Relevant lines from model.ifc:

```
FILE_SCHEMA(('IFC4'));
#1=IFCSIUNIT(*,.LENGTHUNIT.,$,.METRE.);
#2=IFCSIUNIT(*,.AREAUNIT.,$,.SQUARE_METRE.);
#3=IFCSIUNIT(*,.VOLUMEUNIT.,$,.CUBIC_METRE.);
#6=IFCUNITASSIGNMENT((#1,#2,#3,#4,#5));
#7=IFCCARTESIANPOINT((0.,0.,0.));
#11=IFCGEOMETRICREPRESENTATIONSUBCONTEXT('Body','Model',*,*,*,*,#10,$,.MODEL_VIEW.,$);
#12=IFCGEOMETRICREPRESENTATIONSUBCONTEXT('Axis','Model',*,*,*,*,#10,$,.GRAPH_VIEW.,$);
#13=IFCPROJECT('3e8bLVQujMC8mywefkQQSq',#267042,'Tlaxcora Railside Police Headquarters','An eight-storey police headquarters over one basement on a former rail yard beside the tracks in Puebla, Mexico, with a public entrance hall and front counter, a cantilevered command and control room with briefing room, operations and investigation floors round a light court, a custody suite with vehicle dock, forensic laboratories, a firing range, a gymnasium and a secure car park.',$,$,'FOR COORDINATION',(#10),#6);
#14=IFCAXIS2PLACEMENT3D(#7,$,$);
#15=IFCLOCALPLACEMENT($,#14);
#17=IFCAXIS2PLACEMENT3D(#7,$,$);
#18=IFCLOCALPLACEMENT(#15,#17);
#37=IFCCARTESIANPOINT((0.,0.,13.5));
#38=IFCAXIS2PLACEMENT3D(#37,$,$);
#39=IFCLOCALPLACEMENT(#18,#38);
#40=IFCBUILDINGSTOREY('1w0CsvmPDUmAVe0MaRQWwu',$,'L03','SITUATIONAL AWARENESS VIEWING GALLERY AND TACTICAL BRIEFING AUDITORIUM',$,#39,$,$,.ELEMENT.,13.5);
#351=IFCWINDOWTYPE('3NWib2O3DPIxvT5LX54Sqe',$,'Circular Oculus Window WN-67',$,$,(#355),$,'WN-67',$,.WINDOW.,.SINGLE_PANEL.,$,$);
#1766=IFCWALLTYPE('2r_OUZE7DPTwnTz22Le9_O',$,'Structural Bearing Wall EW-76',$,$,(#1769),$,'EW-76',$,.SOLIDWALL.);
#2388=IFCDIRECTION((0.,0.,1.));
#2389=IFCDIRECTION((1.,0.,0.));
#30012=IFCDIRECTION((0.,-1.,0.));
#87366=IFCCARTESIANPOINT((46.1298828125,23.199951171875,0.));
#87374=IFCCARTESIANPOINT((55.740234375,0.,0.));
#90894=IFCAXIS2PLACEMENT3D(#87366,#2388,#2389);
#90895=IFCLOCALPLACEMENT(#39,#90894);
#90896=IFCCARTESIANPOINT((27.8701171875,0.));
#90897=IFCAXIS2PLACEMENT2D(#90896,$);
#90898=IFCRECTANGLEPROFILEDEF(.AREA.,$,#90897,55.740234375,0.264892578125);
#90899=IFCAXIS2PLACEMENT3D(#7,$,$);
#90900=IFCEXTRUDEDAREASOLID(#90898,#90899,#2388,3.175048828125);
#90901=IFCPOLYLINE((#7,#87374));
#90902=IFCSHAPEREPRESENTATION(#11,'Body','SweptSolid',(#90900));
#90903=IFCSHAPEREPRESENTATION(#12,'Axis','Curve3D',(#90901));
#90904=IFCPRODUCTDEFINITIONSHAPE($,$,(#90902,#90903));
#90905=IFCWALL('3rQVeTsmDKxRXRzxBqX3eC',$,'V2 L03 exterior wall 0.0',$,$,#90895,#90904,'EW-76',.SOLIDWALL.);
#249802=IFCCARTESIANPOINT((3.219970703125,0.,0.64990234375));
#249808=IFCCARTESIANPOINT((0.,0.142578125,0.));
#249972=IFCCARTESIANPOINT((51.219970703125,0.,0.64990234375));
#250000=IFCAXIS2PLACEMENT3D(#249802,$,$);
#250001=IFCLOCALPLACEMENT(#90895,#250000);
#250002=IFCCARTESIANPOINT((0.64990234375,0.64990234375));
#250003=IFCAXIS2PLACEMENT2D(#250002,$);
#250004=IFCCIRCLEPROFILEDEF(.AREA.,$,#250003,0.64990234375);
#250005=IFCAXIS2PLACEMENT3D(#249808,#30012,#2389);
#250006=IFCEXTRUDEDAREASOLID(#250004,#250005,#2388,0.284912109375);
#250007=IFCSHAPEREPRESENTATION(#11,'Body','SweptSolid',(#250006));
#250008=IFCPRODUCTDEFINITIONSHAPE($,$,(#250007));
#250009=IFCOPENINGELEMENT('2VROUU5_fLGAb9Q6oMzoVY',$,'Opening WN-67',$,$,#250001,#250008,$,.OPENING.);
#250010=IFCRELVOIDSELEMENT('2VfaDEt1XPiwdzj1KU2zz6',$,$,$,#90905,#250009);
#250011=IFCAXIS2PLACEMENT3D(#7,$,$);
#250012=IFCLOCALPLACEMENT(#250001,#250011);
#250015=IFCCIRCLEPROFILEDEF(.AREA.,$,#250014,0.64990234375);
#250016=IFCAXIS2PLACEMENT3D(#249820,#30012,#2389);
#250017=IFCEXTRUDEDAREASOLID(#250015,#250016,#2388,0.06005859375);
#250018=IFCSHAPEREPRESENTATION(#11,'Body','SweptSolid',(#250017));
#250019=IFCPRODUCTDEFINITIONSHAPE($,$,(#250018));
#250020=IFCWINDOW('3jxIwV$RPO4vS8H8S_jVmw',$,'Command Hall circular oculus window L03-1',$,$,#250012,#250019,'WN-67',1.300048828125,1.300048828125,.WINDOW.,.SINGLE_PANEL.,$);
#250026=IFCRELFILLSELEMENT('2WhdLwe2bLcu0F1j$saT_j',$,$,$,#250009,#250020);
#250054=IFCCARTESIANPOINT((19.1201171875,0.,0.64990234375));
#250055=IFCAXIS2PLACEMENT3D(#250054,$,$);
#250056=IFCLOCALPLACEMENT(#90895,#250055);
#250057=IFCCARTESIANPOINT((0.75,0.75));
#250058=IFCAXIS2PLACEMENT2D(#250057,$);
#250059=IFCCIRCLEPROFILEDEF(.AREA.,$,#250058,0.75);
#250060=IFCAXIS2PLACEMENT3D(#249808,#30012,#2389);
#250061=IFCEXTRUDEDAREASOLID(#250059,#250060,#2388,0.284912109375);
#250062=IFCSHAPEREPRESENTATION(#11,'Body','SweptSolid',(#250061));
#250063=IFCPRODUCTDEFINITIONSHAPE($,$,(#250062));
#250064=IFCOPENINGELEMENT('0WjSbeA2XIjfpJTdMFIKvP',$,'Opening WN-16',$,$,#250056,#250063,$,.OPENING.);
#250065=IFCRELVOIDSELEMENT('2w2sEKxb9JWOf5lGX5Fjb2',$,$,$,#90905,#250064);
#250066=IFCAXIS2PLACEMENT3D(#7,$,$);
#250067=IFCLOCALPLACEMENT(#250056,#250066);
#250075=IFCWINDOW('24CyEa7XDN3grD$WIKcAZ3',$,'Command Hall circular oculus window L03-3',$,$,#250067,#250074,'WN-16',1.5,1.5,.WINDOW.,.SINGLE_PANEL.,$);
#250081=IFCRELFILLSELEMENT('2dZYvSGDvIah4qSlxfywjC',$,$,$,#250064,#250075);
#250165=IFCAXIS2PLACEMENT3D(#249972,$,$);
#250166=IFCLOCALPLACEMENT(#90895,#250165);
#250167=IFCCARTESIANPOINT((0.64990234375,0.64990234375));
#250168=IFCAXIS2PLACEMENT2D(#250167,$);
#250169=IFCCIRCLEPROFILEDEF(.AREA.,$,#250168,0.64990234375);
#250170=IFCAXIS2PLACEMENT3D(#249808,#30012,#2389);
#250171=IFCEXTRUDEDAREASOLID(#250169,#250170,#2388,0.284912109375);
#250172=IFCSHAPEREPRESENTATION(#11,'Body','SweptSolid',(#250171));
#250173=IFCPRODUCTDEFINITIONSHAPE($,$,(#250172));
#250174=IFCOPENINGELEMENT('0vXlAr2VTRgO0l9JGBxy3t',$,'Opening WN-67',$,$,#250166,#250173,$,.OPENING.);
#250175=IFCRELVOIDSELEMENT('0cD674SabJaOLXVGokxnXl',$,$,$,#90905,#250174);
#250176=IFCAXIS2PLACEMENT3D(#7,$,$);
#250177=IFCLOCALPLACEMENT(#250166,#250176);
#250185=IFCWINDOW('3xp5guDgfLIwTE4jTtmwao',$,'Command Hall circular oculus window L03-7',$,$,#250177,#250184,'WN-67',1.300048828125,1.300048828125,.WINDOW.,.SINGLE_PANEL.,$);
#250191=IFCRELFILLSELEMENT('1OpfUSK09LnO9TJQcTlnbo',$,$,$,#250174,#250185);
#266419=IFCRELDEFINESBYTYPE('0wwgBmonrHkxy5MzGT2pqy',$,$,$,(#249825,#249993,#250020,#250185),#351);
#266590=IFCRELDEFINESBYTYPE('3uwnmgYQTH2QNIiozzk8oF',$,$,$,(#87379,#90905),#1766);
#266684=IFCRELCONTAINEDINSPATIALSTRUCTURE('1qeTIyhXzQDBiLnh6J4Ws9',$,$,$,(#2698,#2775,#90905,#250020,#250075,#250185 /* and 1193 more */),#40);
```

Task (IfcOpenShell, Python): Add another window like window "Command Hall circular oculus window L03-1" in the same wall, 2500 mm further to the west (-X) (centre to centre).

```python
import ifcopenshell
import ifcopenshell.api.feature
import ifcopenshell.api.geometry
import ifcopenshell.api.root
import ifcopenshell.geom
import ifcopenshell.util.element
import ifcopenshell.util.placement
import ifcopenshell.util.shape
import ifcopenshell.util.unit

model = ifcopenshell.open("model.ifc")
unit_scale = ifcopenshell.util.unit.calculate_unit_scale(model)
settings = ifcopenshell.geom.settings()


def volume(element):
    """Net volume in cubic metres, openings subtracted."""
    shape = ifcopenshell.geom.create_shape(settings, element)
    return ifcopenshell.util.shape.get_volume(shape.geometry)


window = model.by_guid("3jxIwV$RPO4vS8H8S_jVmw")
opening = window.FillsVoids[0].RelatingOpeningElement
wall = opening.VoidsElements[0].RelatingBuildingElement
before = volume(wall)
shift = ifcopenshell.util.placement.get_local_placement(wall.ObjectPlacement)[:3, 0] * -2.5 / unit_scale

# copy_class copies the void relationship, type, container and properties, but no geometry.
new_opening = ifcopenshell.api.root.copy_class(model, product=opening)
new_opening.Representation = ifcopenshell.util.element.copy_deep(
    model, opening.Representation, exclude=["IfcGeometricRepresentationContext", "IfcRepresentationMap"]
)
new_window = ifcopenshell.api.root.copy_class(model, product=window)
new_window.Representation = ifcopenshell.util.element.copy_deep(
    model, window.Representation, exclude=["IfcGeometricRepresentationContext", "IfcRepresentationMap"]
)
new_window.Tag = None
ifcopenshell.api.feature.add_filling(model, opening=new_opening, element=new_window)

for old, new in ((opening, new_opening), (window, new_window)):
    matrix = ifcopenshell.util.placement.get_local_placement(old.ObjectPlacement)
    matrix[:3, 3] += shift
    ifcopenshell.api.geometry.edit_object_placement(model, product=new, matrix=matrix, is_si=False)

after = volume(wall)

print(f"wall volume {before:.3f} -> {after:.3f} m3")

model.write("model-out.ifc")
```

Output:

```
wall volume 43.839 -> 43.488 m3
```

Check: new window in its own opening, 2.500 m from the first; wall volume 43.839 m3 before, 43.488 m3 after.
